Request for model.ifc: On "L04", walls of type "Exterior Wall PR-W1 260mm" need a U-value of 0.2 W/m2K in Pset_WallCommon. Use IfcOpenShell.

First a look at what the model holds.

```python
import ifcopenshell
import ifcopenshell.util.element

model = ifcopenshell.open("model.ifc")
print(model.schema)
storey = next(s for s in model.by_type("IfcBuildingStorey") if s.Name == "L04")
walls = [e for e in ifcopenshell.util.element.get_decomposition(storey) if e.is_a("IfcWall")]
seen = {}
for e in walls:
    element_type = ifcopenshell.util.element.get_type(e)
    key = (element_type.Name if element_type != e and element_type else None, ifcopenshell.util.element.get_pset(e, "Pset_WallCommon", "ThermalTransmittance"))
    seen[key] = seen.get(key, 0) + 1
for (name, value), count in sorted(seen.items(), key=str):
    print(count, "x", name, "|", value)
```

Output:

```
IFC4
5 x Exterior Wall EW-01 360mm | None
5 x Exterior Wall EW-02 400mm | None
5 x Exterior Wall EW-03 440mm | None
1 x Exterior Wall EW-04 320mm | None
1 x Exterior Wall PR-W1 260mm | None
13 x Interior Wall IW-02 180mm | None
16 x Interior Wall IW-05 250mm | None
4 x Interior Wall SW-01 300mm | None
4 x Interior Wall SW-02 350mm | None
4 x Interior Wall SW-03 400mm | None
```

```python
import ifcopenshell
import ifcopenshell.api.pset
import ifcopenshell.util.element

model = ifcopenshell.open("model.ifc")

storey = next(s for s in model.by_type("IfcBuildingStorey") if s.Name == "L04")
walls = [e for e in ifcopenshell.util.element.get_decomposition(storey) if e.is_a("IfcWall")]

count = 0
for e in walls:
    element_type = ifcopenshell.util.element.get_type(e)
    if element_type in (None, e) or element_type.Name != "Exterior Wall PR-W1 260mm":
        continue
    # add_pset returns the element's existing set when there is one.
    pset = ifcopenshell.api.pset.add_pset(model, product=e, name="Pset_WallCommon")
    ifcopenshell.api.pset.edit_pset(model, pset=pset, properties={"ThermalTransmittance": 0.2})
    count += 1

print(count, "walls updated")

model.write("model-out.ifc")
```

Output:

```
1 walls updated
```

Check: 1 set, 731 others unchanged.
